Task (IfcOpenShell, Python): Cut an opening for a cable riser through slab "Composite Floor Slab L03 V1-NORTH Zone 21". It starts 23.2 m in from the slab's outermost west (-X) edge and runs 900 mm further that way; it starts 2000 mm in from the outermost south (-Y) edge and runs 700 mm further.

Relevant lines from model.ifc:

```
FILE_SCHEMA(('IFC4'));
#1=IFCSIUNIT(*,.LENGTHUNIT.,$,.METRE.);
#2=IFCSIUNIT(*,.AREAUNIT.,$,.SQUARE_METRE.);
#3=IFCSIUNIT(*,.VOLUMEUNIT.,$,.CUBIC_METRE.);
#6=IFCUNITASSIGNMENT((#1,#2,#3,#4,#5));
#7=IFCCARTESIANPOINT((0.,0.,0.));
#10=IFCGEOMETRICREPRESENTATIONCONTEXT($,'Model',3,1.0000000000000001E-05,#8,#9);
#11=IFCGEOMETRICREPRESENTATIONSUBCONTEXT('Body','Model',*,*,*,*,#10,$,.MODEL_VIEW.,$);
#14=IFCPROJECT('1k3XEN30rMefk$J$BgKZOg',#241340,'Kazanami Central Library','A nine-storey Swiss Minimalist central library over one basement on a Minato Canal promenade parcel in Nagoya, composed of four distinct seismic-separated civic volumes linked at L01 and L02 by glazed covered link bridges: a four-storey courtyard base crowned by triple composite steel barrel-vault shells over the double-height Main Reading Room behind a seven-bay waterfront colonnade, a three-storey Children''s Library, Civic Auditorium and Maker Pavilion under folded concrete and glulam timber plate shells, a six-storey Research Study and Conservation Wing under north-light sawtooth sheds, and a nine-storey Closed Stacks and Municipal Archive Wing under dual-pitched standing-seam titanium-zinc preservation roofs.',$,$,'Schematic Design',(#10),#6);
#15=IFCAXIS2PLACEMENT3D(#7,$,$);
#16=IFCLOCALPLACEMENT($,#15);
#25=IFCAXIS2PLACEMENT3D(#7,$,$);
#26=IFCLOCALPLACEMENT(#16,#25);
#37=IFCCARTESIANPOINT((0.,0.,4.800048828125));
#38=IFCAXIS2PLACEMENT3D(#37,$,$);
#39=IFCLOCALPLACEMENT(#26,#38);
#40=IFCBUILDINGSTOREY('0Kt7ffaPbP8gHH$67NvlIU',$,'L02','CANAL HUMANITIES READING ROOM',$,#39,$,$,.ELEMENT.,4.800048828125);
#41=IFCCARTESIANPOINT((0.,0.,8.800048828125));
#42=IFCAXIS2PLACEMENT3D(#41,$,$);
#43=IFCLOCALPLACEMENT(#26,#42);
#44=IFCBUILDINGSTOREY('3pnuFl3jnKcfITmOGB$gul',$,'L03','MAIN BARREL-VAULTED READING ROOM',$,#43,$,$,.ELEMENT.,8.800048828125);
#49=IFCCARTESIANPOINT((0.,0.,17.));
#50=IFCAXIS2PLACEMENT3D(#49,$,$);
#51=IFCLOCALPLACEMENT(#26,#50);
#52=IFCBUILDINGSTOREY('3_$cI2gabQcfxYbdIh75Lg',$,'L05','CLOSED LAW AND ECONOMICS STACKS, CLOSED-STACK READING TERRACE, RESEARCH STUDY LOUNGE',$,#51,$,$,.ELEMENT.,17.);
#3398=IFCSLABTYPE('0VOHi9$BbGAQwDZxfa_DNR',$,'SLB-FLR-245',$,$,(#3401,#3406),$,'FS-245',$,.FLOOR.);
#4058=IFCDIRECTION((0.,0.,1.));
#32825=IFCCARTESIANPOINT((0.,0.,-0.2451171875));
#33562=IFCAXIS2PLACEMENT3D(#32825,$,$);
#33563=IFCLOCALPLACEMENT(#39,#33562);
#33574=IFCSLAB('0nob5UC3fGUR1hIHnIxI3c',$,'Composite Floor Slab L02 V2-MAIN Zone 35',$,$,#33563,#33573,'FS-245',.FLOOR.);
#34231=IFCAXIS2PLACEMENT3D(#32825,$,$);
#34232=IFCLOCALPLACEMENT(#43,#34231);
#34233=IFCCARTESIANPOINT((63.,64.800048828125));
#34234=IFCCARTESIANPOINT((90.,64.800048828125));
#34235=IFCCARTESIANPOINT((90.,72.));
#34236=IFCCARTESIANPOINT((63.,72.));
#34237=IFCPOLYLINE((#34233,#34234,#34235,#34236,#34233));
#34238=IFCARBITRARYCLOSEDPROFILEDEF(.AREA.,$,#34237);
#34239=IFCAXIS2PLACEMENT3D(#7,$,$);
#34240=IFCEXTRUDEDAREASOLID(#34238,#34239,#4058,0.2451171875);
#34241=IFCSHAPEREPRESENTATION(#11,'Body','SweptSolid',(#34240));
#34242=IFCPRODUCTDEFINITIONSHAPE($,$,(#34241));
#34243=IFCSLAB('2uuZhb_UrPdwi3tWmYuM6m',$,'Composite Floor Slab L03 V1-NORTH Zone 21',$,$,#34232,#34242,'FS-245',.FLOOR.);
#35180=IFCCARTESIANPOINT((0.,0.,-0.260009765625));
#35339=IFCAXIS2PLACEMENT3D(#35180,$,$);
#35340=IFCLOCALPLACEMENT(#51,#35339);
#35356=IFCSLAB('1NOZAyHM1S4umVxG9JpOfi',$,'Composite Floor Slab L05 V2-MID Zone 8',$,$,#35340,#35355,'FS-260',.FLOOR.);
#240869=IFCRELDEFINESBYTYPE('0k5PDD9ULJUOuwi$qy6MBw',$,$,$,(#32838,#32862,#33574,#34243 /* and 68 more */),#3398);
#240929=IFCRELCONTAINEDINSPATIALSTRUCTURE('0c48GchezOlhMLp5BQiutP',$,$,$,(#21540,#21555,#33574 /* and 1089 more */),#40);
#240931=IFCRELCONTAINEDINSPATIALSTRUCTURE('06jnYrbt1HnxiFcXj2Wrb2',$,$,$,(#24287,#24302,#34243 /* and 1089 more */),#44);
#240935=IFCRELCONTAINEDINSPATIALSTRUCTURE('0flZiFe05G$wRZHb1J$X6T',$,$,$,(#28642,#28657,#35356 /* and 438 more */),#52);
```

```python
import numpy as np
import ifcopenshell
import ifcopenshell.api.feature
import ifcopenshell.api.geometry
import ifcopenshell.api.root
import ifcopenshell.geom
import ifcopenshell.util.placement
import ifcopenshell.util.representation
import ifcopenshell.util.shape
import ifcopenshell.util.unit

model = ifcopenshell.open("model.ifc")
unit_scale = ifcopenshell.util.unit.calculate_unit_scale(model)
settings = ifcopenshell.geom.settings()


def volume(element):
    """Net volume in cubic metres, openings subtracted."""
    shape = ifcopenshell.geom.create_shape(settings, element)
    return ifcopenshell.util.shape.get_volume(shape.geometry)


slab = model.by_guid("2uuZhb_UrPdwi3tWmYuM6m")
before = volume(slab)

# Extent in the slab's own axes, in metres. The edges named are its -X and -Y sides.
slab_shape = ifcopenshell.geom.create_shape(settings, slab)
vertices = ifcopenshell.util.shape.get_vertices(slab_shape.geometry)
x_min, y_min, bottom = vertices.min(axis=0)
top = vertices[:, 2].max()

opening = ifcopenshell.api.root.create_entity(model, ifc_class="IfcOpeningElement", name="Cable riser opening", predefined_type="OPENING")
context = ifcopenshell.util.representation.get_context(model, "Model", "Body", "MODEL_VIEW")
width, depth = 0.9, 0.7
outline = [(0.0, 0.0), (width, 0.0), (width, depth), (0.0, depth), (0.0, 0.0)]
# Overshoot both faces by 50 mm so the cut is clean.
shape = ifcopenshell.api.geometry.add_slab_representation(
    model, context=context, depth=top - bottom + 0.1, polyline=outline
)
ifcopenshell.api.geometry.assign_representation(model, product=opening, representation=shape)

matrix = ifcopenshell.util.placement.get_local_placement(slab.ObjectPlacement)
matrix[:, 3] = matrix @ np.append(np.array([x_min + 23.2, y_min + 2, bottom - 0.05]) / unit_scale, 1.0)
ifcopenshell.api.geometry.edit_object_placement(model, product=opening, matrix=matrix, is_si=False)
ifcopenshell.api.feature.add_feature(model, feature=opening, element=slab)

after = volume(slab)

print(f"slab volume {before:.3f} -> {after:.3f} m3")

model.write("model_rev.ifc")
```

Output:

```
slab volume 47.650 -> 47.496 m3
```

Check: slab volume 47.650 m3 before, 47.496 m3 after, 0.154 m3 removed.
